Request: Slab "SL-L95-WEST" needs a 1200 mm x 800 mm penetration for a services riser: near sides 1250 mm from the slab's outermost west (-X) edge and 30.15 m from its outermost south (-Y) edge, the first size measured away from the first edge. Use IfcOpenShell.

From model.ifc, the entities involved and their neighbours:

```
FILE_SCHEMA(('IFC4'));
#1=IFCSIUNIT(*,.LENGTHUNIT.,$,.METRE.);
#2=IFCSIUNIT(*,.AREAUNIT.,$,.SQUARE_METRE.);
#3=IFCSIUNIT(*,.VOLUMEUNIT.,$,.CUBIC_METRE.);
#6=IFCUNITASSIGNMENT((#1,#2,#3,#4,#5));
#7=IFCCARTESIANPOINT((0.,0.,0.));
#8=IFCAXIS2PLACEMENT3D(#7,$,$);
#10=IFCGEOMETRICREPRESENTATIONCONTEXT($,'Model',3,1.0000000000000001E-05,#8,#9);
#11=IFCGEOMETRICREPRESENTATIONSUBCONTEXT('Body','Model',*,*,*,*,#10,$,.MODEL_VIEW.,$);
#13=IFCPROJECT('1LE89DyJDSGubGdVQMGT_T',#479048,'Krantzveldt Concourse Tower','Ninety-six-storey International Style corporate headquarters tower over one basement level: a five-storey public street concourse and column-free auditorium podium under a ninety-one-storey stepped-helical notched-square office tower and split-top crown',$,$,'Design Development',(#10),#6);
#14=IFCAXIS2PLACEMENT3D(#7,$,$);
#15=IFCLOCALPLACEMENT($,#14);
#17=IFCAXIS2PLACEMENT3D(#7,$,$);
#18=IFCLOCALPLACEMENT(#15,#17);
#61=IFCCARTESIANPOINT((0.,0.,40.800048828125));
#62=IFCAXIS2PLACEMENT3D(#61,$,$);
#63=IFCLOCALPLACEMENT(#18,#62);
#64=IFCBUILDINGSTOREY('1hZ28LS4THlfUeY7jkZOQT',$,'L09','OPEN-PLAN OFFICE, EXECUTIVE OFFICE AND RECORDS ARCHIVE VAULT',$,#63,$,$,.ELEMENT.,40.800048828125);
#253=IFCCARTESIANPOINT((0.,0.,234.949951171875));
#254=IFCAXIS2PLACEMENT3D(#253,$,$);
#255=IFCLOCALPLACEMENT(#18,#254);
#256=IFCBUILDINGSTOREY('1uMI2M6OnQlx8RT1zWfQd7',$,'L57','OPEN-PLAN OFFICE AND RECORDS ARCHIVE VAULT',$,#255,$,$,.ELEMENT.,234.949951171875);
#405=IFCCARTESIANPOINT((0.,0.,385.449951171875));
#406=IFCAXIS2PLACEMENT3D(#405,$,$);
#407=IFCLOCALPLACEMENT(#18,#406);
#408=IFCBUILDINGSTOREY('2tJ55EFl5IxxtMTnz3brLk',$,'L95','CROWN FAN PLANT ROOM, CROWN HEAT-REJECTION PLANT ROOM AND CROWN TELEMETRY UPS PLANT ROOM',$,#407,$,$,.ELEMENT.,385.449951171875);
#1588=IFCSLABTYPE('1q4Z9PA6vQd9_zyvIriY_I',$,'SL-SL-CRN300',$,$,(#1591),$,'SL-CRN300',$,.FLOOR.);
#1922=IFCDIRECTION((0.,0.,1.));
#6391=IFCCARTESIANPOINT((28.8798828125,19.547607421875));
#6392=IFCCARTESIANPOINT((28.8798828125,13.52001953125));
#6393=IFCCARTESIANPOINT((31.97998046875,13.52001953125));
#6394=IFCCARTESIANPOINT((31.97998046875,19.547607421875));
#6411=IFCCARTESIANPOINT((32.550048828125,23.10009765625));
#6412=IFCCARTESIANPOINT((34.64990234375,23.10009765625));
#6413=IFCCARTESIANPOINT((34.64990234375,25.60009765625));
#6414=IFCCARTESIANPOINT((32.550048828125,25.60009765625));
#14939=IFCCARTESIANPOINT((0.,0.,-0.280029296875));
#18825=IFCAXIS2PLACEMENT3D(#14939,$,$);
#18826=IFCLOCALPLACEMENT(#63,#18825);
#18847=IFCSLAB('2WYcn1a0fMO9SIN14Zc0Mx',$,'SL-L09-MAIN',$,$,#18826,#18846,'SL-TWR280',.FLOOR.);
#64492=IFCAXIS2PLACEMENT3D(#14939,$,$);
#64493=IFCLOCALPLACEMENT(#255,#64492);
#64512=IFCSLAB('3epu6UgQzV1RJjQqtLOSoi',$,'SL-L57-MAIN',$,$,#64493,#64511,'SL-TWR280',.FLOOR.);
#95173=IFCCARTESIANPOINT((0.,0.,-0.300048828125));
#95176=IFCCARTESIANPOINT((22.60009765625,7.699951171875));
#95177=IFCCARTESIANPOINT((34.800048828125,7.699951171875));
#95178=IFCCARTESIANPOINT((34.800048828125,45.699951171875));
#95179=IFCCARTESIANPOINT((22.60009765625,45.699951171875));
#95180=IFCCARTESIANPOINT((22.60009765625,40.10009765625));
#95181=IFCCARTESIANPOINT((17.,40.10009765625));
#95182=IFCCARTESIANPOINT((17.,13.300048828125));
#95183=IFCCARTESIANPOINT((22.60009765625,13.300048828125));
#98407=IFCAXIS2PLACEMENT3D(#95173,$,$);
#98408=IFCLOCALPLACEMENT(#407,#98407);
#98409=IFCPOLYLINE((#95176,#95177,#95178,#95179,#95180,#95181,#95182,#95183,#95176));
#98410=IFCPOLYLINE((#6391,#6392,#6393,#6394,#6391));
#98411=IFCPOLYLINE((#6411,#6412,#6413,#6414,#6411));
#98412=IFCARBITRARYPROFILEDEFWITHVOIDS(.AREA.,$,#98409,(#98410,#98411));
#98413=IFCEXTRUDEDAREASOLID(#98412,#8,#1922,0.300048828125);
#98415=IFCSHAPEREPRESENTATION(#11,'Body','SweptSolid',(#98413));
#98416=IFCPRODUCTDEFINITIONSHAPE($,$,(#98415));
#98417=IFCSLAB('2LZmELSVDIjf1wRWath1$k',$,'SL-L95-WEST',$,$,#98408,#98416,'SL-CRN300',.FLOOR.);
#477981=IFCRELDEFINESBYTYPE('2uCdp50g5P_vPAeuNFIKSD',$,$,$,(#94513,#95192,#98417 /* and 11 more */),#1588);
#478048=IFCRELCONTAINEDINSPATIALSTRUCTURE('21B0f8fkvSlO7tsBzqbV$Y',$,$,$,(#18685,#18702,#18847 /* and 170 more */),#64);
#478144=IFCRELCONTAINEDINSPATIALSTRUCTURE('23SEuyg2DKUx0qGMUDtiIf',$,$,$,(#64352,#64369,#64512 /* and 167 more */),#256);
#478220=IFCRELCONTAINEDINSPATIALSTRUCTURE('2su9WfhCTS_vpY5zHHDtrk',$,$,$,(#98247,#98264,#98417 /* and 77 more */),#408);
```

```python
import numpy as np
import ifcopenshell
import ifcopenshell.api.feature
import ifcopenshell.api.geometry
import ifcopenshell.api.root
import ifcopenshell.geom
import ifcopenshell.util.placement
import ifcopenshell.util.representation
import ifcopenshell.util.shape
import ifcopenshell.util.unit

model = ifcopenshell.open("model.ifc")
unit_scale = ifcopenshell.util.unit.calculate_unit_scale(model)
settings = ifcopenshell.geom.settings()


def volume(element):
    """Net volume in cubic metres, openings subtracted."""
    shape = ifcopenshell.geom.create_shape(settings, element)
    return ifcopenshell.util.shape.get_volume(shape.geometry)


slab = model.by_guid("2LZmELSVDIjf1wRWath1$k")
before = volume(slab)

# Extent in the slab's own axes, in metres. The edges named are its -X and -Y sides.
slab_shape = ifcopenshell.geom.create_shape(settings, slab)
vertices = ifcopenshell.util.shape.get_vertices(slab_shape.geometry)
x_min, y_min, bottom = vertices.min(axis=0)
top = vertices[:, 2].max()

opening = ifcopenshell.api.root.create_entity(model, ifc_class="IfcOpeningElement", name="Services riser opening", predefined_type="OPENING")
context = ifcopenshell.util.representation.get_context(model, "Model", "Body", "MODEL_VIEW")
width, depth = 1.2, 0.8
outline = [(0.0, 0.0), (width, 0.0), (width, depth), (0.0, depth), (0.0, 0.0)]
# Overshoot both faces by 50 mm so the cut is clean.
shape = ifcopenshell.api.geometry.add_slab_representation(
    model, context=context, depth=top - bottom + 0.1, polyline=outline
)
ifcopenshell.api.geometry.assign_representation(model, product=opening, representation=shape)

matrix = ifcopenshell.util.placement.get_local_placement(slab.ObjectPlacement)
matrix[:, 3] = matrix @ np.append(np.array([x_min + 1.25, y_min + 30.15, bottom - 0.05]) / unit_scale, 1.0)
ifcopenshell.api.geometry.edit_object_placement(model, product=opening, matrix=matrix, is_si=False)
ifcopenshell.api.feature.add_feature(model, feature=opening, element=slab)

after = volume(slab)

print(f"slab volume {before:.3f} -> {after:.3f} m3")

model.write("model_edited.ifc")
```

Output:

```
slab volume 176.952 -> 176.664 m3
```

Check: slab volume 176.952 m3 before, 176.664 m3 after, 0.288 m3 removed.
